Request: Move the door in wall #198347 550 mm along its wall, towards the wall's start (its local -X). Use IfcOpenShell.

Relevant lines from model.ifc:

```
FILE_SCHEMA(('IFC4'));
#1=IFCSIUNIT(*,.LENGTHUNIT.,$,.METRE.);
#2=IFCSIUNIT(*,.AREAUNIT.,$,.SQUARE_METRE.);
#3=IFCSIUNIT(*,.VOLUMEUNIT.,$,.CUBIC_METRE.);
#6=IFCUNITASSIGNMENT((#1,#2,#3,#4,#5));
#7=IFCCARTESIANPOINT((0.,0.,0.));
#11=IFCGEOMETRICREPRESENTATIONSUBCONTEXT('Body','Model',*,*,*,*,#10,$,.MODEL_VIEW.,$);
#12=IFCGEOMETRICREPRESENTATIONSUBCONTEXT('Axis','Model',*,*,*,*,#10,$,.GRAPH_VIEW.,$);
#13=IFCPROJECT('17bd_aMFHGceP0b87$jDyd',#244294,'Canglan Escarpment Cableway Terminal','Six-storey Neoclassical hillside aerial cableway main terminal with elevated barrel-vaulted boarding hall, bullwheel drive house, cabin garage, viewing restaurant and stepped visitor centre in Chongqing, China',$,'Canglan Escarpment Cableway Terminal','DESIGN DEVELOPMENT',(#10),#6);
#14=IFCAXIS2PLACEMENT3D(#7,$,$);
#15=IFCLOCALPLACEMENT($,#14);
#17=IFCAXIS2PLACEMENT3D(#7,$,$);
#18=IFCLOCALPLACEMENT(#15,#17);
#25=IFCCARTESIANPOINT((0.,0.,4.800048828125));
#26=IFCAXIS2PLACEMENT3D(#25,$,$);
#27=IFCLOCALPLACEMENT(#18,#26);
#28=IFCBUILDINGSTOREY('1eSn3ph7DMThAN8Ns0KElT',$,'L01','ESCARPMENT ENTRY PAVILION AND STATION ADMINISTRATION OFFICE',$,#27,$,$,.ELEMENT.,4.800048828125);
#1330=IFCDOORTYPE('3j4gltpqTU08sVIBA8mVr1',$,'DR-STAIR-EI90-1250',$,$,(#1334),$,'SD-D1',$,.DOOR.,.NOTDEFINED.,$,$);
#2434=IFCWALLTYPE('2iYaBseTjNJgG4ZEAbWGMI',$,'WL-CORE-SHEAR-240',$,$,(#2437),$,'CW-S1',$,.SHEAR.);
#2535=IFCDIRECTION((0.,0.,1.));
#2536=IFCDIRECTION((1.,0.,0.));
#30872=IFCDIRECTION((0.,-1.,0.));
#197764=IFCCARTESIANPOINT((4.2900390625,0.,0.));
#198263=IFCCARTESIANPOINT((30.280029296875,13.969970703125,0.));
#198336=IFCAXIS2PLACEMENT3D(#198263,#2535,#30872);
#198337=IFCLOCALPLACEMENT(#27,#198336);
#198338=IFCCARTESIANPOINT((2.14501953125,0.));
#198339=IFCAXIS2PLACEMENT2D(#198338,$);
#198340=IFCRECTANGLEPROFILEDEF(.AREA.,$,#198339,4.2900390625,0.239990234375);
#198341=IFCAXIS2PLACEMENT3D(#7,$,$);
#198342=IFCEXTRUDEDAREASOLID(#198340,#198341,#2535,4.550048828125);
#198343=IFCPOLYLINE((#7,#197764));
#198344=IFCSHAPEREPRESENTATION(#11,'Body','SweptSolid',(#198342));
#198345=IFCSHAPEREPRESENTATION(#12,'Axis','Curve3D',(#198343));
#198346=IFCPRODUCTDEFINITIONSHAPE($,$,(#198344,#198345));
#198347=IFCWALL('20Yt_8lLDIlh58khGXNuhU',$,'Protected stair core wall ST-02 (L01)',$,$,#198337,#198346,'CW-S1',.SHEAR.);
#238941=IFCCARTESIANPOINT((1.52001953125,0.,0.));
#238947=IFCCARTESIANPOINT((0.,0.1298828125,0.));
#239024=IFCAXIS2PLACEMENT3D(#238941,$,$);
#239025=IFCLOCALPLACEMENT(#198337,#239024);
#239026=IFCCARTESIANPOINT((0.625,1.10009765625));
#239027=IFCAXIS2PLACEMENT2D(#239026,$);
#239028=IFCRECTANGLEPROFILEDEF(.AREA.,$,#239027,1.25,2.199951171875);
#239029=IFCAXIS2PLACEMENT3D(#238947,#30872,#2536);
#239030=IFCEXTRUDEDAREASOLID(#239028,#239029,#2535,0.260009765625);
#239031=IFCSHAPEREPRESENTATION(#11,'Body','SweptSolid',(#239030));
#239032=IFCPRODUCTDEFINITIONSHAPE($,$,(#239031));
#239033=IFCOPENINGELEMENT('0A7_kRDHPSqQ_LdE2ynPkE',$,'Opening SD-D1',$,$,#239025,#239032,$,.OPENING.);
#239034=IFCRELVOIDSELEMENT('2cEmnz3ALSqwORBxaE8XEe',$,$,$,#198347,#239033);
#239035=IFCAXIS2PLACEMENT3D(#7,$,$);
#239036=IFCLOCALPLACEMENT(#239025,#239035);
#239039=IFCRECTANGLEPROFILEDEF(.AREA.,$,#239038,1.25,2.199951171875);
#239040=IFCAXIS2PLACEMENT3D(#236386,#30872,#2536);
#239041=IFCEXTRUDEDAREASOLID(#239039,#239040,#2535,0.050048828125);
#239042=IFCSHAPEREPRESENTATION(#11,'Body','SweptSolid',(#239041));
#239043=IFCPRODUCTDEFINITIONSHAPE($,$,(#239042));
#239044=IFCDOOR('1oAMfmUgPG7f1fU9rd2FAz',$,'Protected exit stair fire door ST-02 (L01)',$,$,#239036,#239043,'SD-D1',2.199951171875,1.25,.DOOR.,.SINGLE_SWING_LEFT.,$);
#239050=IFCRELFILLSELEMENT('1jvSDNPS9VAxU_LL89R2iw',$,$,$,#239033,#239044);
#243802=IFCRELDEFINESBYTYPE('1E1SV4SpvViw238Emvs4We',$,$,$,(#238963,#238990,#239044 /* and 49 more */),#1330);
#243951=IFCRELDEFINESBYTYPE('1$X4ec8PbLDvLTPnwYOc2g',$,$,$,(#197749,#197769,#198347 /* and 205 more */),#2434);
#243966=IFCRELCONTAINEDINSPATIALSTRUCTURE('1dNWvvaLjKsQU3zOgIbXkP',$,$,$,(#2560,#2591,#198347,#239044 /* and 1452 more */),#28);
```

```python
import ifcopenshell
import ifcopenshell.api.geometry
import ifcopenshell.util.placement
import ifcopenshell.util.unit

model = ifcopenshell.open("model.ifc")
unit_scale = ifcopenshell.util.unit.calculate_unit_scale(model)

door = model.by_id(239044)
opening = door.FillsVoids[0].RelatingOpeningElement
wall = opening.VoidsElements[0].RelatingBuildingElement

wall_matrix = ifcopenshell.util.placement.get_local_placement(wall.ObjectPlacement)
shift = wall_matrix[:3, 0] * -0.55 / unit_scale
before = ifcopenshell.util.placement.get_local_placement(door.ObjectPlacement)[:3, 3].copy()

# The door is placed relative to its opening, so it follows when the opening moves.
matrix = ifcopenshell.util.placement.get_local_placement(opening.ObjectPlacement)
matrix[:3, 3] += shift
ifcopenshell.api.geometry.edit_object_placement(
    model, product=opening, matrix=matrix, is_si=False, should_transform_children=True
)

after = ifcopenshell.util.placement.get_local_placement(door.ObjectPlacement)[:3, 3]
print("door moved by", (after - before).round(3) + 0.0)

model.write("model_rev.ifc")
```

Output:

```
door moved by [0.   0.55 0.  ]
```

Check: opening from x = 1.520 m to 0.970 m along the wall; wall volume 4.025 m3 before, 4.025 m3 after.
